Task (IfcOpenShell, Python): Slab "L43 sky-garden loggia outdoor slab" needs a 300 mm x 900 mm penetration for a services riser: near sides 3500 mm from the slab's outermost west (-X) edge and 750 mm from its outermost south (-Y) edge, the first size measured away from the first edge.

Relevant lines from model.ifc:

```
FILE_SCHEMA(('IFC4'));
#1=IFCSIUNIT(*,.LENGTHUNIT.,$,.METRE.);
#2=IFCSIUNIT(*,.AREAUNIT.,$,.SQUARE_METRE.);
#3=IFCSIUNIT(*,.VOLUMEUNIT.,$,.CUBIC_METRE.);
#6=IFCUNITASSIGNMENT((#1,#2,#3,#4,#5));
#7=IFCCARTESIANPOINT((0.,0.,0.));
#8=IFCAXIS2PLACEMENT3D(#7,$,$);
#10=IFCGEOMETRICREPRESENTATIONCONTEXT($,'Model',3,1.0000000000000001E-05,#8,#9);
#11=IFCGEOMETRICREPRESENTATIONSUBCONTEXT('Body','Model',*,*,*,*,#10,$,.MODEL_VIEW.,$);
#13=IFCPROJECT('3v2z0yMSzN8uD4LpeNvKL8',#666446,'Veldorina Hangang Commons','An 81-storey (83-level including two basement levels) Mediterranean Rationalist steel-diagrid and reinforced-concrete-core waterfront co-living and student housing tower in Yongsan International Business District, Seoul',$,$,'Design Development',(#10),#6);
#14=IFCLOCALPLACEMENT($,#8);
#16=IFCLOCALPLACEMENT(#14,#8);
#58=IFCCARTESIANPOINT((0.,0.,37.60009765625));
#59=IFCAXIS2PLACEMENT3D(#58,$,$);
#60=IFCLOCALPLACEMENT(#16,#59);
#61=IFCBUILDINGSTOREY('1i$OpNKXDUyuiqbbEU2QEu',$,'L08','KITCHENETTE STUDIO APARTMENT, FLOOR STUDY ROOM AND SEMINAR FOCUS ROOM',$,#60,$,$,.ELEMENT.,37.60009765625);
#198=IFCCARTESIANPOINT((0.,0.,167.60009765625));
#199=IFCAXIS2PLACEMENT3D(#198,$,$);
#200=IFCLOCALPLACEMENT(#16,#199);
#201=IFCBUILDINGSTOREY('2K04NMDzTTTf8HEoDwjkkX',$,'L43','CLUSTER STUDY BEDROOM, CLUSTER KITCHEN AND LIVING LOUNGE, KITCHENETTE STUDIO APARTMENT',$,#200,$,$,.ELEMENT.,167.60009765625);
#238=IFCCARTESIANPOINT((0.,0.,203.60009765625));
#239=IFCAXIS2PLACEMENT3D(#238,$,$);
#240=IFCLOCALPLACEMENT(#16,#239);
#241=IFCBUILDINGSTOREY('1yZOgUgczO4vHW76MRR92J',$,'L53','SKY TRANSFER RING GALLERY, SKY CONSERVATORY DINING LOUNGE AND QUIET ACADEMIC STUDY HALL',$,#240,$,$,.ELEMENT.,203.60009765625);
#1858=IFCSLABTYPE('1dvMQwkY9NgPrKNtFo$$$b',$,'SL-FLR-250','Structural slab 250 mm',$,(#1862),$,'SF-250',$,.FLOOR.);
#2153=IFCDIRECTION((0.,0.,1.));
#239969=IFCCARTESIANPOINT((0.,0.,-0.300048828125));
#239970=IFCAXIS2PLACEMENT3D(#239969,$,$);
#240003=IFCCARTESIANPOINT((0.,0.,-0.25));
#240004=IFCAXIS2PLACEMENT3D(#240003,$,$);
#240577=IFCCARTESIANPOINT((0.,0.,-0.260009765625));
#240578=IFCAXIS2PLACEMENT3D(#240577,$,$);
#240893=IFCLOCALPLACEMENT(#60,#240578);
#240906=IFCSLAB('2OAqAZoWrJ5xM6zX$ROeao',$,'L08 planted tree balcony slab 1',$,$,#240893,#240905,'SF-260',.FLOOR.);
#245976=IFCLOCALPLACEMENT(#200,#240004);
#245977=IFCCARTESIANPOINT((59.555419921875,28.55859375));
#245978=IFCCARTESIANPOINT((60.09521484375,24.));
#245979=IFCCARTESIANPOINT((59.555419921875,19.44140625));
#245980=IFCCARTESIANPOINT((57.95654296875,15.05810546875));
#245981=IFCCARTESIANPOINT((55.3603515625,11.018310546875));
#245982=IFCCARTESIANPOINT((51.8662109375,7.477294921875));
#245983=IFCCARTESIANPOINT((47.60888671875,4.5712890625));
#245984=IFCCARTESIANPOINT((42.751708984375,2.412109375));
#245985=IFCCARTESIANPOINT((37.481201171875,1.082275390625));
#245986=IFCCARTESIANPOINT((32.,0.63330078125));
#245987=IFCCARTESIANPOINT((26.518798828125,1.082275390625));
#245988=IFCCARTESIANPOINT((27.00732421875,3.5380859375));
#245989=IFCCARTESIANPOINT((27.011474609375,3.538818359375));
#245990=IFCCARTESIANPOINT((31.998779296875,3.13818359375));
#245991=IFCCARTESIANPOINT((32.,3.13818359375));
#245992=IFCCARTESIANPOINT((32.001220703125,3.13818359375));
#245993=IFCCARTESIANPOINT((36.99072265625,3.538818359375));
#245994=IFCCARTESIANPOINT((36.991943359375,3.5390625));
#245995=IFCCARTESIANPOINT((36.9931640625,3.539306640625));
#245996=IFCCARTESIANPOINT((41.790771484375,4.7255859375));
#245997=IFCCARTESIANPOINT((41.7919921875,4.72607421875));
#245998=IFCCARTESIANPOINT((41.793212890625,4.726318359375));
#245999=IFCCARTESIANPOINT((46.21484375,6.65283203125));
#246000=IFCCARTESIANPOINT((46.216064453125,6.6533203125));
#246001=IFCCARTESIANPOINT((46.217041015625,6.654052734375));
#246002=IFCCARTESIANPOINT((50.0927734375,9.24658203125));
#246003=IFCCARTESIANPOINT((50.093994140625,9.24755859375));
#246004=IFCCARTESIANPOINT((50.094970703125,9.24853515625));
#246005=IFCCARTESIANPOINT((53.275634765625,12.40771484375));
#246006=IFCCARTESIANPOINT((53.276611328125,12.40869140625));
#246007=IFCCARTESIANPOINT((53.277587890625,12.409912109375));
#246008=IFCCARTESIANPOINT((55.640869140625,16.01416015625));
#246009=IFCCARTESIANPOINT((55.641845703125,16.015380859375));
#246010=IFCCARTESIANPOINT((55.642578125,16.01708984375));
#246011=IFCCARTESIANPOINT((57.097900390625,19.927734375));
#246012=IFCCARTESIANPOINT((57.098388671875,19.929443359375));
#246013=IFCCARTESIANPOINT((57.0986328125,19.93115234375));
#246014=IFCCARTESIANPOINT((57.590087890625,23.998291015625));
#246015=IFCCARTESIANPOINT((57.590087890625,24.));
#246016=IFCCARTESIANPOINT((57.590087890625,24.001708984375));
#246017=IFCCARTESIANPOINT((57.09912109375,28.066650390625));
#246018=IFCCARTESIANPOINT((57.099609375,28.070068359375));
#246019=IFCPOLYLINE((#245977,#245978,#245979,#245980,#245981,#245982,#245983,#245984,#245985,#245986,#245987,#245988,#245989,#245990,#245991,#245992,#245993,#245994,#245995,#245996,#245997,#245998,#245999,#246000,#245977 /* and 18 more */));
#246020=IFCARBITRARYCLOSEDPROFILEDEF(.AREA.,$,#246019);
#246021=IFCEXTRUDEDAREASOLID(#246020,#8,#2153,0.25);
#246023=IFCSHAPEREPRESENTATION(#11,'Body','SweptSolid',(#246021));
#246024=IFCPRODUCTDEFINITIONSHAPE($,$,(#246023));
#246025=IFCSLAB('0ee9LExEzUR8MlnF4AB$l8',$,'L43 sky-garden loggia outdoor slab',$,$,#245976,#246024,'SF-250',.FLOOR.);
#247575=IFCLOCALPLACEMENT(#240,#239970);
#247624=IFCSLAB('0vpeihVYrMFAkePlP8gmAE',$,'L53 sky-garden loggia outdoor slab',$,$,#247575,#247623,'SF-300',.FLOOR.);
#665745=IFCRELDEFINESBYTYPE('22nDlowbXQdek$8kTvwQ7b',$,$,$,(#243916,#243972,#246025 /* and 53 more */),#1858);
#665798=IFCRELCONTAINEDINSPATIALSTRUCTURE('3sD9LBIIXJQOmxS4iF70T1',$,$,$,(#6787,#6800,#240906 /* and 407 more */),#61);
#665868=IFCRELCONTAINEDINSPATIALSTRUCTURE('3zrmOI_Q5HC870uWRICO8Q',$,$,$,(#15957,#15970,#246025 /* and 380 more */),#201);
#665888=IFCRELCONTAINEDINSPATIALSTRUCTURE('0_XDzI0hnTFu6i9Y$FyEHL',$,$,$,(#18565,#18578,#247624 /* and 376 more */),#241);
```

```python
import numpy as np
import ifcopenshell
import ifcopenshell.api.feature
import ifcopenshell.api.geometry
import ifcopenshell.api.root
import ifcopenshell.geom
import ifcopenshell.util.placement
import ifcopenshell.util.representation
import ifcopenshell.util.shape
import ifcopenshell.util.unit

model = ifcopenshell.open("model.ifc")
unit_scale = ifcopenshell.util.unit.calculate_unit_scale(model)
settings = ifcopenshell.geom.settings()


def volume(element):
    """Net volume in cubic metres, openings subtracted."""
    shape = ifcopenshell.geom.create_shape(settings, element)
    return ifcopenshell.util.shape.get_volume(shape.geometry)


slab = model.by_guid("0ee9LExEzUR8MlnF4AB$l8")
before = volume(slab)

# Extent in the slab's own axes, in metres. The edges named are its -X and -Y sides.
slab_shape = ifcopenshell.geom.create_shape(settings, slab)
vertices = ifcopenshell.util.shape.get_vertices(slab_shape.geometry)
x_min, y_min, bottom = vertices.min(axis=0)
top = vertices[:, 2].max()

opening = ifcopenshell.api.root.create_entity(model, ifc_class="IfcOpeningElement", name="Services riser opening", predefined_type="OPENING")
context = ifcopenshell.util.representation.get_context(model, "Model", "Body", "MODEL_VIEW")
width, depth = 0.3, 0.9
outline = [(0.0, 0.0), (width, 0.0), (width, depth), (0.0, depth), (0.0, 0.0)]
# Overshoot both faces by 50 mm so the cut is clean.
shape = ifcopenshell.api.geometry.add_slab_representation(
    model, context=context, depth=top - bottom + 0.1, polyline=outline
)
ifcopenshell.api.geometry.assign_representation(model, product=opening, representation=shape)

matrix = ifcopenshell.util.placement.get_local_placement(slab.ObjectPlacement)
matrix[:, 3] = matrix @ np.append(np.array([x_min + 3.5, y_min + 0.75, bottom - 0.05]) / unit_scale, 1.0)
ifcopenshell.api.geometry.edit_object_placement(model, product=opening, matrix=matrix, is_si=False)
ifcopenshell.api.feature.add_feature(model, feature=opening, element=slab)

after = volume(slab)

print(f"slab volume {before:.3f} -> {after:.3f} m3")

model.write("model_edited.ifc")
```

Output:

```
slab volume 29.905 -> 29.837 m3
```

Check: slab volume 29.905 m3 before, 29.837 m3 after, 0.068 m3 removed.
